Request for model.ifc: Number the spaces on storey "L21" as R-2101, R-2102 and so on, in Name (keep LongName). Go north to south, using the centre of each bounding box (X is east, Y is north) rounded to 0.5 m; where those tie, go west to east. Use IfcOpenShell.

First a look at what the model holds.

```python
import ifcopenshell
import ifcopenshell.util.element
import ifcopenshell.util.placement

model = ifcopenshell.open("model.ifc")
print(model.schema)
storey = next(s for s in model.by_type("IfcBuildingStorey") if s.Name == "L21")
spaces = [e for e in ifcopenshell.util.element.get_decomposition(storey) if e.is_a("IfcSpace")]
for e in sorted(spaces, key=lambda e: e.id()):
    origin = ifcopenshell.util.placement.get_local_placement(e.ObjectPlacement)[:3, 3]
    print(e.id(), e.Name, e.LongName, origin.round(2) + 0.0, sep=" | ")
```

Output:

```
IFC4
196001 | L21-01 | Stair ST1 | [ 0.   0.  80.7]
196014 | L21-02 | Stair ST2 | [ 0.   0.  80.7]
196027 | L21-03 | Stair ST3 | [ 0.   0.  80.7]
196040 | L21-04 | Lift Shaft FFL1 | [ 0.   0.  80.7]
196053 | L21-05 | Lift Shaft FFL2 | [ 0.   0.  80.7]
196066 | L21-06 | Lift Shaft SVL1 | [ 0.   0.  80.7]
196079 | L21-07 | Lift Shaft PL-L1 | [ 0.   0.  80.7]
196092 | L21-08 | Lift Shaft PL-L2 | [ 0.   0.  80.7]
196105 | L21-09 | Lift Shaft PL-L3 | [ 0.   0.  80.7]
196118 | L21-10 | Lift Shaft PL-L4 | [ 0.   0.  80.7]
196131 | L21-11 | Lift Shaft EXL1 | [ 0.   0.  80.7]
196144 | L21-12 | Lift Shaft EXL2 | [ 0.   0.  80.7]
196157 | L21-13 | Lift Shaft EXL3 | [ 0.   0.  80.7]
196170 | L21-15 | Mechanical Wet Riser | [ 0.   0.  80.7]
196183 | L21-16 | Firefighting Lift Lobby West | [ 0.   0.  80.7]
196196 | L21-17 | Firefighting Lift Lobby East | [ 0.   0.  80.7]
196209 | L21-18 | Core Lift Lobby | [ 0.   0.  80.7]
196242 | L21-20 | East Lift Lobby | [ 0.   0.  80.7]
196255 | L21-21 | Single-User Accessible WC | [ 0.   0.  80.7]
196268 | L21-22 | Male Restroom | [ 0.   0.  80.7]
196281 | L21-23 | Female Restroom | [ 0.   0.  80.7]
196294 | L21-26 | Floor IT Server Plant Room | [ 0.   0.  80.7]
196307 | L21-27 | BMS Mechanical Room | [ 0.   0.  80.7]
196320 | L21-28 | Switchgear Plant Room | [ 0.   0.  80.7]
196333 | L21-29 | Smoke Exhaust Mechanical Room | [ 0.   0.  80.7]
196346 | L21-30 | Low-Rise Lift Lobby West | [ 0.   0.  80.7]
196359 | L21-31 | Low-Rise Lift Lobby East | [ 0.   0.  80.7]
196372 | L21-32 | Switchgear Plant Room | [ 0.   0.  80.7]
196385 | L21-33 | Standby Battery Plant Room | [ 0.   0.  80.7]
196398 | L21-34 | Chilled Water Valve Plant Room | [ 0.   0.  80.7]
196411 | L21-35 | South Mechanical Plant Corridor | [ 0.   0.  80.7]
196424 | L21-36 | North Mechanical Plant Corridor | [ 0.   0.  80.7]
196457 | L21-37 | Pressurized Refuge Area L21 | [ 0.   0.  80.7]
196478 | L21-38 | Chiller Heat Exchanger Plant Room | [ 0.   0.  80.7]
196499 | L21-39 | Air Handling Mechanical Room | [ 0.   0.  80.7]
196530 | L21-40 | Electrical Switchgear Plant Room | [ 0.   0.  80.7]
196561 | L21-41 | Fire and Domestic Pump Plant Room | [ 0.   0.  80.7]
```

```python
import ifcopenshell
import ifcopenshell.geom
import ifcopenshell.util.element
import ifcopenshell.util.shape

model = ifcopenshell.open("model.ifc")
settings = ifcopenshell.geom.settings()
settings.set("use-world-coords", True)


def centre(element):
    shape = ifcopenshell.geom.create_shape(settings, element)
    return ifcopenshell.util.shape.get_bbox_centroid(shape.geometry)


storey = next(s for s in model.by_type("IfcBuildingStorey") if s.Name == "L21")
spaces = [e for e in ifcopenshell.util.element.get_decomposition(storey) if e.is_a("IfcSpace")]

# Insertion points can sit at a corner or the storey origin, so sort by the geometry (in metres).
centres = {e: centre(e) for e in spaces}
spaces.sort(key=lambda e: (-round(centres[e][1] / 0.5), centres[e][0]))

for i, e in enumerate(spaces, start=1):
    number = f"R-21{i:02d}"
    e.Name = number
    print(e.id(), number)

model.write("model_rev.ifc")
```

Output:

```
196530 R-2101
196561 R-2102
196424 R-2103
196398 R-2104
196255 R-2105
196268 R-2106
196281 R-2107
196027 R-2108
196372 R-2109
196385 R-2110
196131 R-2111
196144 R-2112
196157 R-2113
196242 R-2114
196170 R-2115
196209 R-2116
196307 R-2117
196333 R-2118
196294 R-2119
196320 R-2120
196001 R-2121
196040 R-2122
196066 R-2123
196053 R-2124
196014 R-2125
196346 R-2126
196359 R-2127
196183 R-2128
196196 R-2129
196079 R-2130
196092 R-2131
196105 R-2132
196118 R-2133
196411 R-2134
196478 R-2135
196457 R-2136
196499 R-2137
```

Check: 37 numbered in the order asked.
